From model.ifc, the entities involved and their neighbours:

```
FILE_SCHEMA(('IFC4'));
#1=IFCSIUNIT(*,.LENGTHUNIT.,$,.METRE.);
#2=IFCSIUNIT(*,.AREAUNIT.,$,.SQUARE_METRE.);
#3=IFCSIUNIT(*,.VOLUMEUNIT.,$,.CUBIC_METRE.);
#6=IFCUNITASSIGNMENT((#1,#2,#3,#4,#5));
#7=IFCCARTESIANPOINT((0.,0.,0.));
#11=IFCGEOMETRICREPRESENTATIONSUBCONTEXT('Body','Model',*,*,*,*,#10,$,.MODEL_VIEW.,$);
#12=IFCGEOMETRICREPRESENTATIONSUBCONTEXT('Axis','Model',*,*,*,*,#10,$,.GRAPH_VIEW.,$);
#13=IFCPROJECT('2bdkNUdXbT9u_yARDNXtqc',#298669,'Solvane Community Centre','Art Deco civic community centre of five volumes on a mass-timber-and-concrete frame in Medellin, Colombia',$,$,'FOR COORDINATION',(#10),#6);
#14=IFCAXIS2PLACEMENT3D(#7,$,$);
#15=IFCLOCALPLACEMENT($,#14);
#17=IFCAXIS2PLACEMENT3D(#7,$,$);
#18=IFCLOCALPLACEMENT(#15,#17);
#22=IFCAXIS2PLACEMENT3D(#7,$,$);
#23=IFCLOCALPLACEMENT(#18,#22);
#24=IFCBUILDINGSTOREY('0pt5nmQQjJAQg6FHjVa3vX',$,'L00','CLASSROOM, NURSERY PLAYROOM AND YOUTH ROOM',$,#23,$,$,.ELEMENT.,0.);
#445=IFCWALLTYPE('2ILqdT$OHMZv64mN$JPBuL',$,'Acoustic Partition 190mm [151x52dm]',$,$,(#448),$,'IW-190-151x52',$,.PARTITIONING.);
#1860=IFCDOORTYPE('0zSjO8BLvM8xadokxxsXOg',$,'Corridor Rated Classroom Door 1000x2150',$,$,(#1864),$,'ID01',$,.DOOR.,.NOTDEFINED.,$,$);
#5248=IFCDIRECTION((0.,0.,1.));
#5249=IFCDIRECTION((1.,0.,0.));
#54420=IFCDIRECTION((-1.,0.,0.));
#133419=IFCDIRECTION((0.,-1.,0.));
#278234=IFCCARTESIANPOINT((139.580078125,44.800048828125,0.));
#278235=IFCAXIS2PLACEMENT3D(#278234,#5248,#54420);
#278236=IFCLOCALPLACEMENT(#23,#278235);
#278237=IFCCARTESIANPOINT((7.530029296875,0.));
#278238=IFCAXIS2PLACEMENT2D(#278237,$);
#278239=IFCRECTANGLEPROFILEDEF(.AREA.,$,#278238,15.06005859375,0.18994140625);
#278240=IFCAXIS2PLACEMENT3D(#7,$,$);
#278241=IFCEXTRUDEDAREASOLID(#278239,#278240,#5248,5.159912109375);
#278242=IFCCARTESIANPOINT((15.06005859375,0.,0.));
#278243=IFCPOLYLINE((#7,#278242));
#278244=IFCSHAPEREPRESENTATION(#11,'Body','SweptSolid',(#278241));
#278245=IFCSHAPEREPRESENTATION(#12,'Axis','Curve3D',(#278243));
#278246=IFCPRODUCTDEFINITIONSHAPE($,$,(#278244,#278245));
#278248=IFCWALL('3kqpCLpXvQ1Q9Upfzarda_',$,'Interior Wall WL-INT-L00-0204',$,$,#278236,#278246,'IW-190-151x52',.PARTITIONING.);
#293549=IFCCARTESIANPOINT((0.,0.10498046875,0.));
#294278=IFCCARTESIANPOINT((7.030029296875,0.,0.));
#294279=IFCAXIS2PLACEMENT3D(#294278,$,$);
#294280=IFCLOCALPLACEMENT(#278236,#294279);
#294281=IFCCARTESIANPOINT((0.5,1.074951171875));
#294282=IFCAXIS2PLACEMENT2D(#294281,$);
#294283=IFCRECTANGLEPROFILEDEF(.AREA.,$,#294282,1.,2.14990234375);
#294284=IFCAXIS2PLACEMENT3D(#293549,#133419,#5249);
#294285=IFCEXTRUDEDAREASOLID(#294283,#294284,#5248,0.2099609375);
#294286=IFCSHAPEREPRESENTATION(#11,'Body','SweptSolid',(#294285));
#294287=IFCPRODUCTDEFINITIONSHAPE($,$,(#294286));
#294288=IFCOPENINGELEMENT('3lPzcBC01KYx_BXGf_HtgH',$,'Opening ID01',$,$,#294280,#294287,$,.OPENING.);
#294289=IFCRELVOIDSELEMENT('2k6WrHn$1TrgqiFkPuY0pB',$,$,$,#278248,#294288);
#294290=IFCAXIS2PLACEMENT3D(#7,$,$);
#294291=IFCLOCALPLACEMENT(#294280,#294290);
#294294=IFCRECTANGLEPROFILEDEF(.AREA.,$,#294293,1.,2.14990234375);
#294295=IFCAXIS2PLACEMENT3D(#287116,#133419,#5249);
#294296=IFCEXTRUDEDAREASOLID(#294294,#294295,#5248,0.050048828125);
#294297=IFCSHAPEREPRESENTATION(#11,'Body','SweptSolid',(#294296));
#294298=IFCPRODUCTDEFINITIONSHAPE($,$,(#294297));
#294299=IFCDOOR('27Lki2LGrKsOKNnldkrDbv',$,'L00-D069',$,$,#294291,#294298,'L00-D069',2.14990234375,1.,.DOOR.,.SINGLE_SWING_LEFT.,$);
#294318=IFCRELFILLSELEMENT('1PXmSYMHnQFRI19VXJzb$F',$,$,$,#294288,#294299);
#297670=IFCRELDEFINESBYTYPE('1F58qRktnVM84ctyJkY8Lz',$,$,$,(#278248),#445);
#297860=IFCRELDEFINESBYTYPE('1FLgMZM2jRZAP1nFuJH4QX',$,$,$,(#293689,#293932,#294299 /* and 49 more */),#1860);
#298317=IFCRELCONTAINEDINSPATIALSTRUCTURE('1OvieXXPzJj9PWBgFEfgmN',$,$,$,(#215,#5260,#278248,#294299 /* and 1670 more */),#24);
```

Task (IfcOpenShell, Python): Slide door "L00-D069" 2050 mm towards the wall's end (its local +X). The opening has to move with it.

```python
import ifcopenshell
import ifcopenshell.api.geometry
import ifcopenshell.util.placement
import ifcopenshell.util.unit

model = ifcopenshell.open("model.ifc")
unit_scale = ifcopenshell.util.unit.calculate_unit_scale(model)

door = model.by_guid("27Lki2LGrKsOKNnldkrDbv")
opening = door.FillsVoids[0].RelatingOpeningElement
wall = opening.VoidsElements[0].RelatingBuildingElement

wall_matrix = ifcopenshell.util.placement.get_local_placement(wall.ObjectPlacement)
shift = wall_matrix[:3, 0] * 2.05 / unit_scale
before = ifcopenshell.util.placement.get_local_placement(door.ObjectPlacement)[:3, 3].copy()

# The door is placed relative to its opening, so it follows when the opening moves.
matrix = ifcopenshell.util.placement.get_local_placement(opening.ObjectPlacement)
matrix[:3, 3] += shift
ifcopenshell.api.geometry.edit_object_placement(
    model, product=opening, matrix=matrix, is_si=False, should_transform_children=True
)

after = ifcopenshell.util.placement.get_local_placement(door.ObjectPlacement)[:3, 3]
print("door moved by", (after - before).round(3) + 0.0)

model.write("model-out.ifc")
```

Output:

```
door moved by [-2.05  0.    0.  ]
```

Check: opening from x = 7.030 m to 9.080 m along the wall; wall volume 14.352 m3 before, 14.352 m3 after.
